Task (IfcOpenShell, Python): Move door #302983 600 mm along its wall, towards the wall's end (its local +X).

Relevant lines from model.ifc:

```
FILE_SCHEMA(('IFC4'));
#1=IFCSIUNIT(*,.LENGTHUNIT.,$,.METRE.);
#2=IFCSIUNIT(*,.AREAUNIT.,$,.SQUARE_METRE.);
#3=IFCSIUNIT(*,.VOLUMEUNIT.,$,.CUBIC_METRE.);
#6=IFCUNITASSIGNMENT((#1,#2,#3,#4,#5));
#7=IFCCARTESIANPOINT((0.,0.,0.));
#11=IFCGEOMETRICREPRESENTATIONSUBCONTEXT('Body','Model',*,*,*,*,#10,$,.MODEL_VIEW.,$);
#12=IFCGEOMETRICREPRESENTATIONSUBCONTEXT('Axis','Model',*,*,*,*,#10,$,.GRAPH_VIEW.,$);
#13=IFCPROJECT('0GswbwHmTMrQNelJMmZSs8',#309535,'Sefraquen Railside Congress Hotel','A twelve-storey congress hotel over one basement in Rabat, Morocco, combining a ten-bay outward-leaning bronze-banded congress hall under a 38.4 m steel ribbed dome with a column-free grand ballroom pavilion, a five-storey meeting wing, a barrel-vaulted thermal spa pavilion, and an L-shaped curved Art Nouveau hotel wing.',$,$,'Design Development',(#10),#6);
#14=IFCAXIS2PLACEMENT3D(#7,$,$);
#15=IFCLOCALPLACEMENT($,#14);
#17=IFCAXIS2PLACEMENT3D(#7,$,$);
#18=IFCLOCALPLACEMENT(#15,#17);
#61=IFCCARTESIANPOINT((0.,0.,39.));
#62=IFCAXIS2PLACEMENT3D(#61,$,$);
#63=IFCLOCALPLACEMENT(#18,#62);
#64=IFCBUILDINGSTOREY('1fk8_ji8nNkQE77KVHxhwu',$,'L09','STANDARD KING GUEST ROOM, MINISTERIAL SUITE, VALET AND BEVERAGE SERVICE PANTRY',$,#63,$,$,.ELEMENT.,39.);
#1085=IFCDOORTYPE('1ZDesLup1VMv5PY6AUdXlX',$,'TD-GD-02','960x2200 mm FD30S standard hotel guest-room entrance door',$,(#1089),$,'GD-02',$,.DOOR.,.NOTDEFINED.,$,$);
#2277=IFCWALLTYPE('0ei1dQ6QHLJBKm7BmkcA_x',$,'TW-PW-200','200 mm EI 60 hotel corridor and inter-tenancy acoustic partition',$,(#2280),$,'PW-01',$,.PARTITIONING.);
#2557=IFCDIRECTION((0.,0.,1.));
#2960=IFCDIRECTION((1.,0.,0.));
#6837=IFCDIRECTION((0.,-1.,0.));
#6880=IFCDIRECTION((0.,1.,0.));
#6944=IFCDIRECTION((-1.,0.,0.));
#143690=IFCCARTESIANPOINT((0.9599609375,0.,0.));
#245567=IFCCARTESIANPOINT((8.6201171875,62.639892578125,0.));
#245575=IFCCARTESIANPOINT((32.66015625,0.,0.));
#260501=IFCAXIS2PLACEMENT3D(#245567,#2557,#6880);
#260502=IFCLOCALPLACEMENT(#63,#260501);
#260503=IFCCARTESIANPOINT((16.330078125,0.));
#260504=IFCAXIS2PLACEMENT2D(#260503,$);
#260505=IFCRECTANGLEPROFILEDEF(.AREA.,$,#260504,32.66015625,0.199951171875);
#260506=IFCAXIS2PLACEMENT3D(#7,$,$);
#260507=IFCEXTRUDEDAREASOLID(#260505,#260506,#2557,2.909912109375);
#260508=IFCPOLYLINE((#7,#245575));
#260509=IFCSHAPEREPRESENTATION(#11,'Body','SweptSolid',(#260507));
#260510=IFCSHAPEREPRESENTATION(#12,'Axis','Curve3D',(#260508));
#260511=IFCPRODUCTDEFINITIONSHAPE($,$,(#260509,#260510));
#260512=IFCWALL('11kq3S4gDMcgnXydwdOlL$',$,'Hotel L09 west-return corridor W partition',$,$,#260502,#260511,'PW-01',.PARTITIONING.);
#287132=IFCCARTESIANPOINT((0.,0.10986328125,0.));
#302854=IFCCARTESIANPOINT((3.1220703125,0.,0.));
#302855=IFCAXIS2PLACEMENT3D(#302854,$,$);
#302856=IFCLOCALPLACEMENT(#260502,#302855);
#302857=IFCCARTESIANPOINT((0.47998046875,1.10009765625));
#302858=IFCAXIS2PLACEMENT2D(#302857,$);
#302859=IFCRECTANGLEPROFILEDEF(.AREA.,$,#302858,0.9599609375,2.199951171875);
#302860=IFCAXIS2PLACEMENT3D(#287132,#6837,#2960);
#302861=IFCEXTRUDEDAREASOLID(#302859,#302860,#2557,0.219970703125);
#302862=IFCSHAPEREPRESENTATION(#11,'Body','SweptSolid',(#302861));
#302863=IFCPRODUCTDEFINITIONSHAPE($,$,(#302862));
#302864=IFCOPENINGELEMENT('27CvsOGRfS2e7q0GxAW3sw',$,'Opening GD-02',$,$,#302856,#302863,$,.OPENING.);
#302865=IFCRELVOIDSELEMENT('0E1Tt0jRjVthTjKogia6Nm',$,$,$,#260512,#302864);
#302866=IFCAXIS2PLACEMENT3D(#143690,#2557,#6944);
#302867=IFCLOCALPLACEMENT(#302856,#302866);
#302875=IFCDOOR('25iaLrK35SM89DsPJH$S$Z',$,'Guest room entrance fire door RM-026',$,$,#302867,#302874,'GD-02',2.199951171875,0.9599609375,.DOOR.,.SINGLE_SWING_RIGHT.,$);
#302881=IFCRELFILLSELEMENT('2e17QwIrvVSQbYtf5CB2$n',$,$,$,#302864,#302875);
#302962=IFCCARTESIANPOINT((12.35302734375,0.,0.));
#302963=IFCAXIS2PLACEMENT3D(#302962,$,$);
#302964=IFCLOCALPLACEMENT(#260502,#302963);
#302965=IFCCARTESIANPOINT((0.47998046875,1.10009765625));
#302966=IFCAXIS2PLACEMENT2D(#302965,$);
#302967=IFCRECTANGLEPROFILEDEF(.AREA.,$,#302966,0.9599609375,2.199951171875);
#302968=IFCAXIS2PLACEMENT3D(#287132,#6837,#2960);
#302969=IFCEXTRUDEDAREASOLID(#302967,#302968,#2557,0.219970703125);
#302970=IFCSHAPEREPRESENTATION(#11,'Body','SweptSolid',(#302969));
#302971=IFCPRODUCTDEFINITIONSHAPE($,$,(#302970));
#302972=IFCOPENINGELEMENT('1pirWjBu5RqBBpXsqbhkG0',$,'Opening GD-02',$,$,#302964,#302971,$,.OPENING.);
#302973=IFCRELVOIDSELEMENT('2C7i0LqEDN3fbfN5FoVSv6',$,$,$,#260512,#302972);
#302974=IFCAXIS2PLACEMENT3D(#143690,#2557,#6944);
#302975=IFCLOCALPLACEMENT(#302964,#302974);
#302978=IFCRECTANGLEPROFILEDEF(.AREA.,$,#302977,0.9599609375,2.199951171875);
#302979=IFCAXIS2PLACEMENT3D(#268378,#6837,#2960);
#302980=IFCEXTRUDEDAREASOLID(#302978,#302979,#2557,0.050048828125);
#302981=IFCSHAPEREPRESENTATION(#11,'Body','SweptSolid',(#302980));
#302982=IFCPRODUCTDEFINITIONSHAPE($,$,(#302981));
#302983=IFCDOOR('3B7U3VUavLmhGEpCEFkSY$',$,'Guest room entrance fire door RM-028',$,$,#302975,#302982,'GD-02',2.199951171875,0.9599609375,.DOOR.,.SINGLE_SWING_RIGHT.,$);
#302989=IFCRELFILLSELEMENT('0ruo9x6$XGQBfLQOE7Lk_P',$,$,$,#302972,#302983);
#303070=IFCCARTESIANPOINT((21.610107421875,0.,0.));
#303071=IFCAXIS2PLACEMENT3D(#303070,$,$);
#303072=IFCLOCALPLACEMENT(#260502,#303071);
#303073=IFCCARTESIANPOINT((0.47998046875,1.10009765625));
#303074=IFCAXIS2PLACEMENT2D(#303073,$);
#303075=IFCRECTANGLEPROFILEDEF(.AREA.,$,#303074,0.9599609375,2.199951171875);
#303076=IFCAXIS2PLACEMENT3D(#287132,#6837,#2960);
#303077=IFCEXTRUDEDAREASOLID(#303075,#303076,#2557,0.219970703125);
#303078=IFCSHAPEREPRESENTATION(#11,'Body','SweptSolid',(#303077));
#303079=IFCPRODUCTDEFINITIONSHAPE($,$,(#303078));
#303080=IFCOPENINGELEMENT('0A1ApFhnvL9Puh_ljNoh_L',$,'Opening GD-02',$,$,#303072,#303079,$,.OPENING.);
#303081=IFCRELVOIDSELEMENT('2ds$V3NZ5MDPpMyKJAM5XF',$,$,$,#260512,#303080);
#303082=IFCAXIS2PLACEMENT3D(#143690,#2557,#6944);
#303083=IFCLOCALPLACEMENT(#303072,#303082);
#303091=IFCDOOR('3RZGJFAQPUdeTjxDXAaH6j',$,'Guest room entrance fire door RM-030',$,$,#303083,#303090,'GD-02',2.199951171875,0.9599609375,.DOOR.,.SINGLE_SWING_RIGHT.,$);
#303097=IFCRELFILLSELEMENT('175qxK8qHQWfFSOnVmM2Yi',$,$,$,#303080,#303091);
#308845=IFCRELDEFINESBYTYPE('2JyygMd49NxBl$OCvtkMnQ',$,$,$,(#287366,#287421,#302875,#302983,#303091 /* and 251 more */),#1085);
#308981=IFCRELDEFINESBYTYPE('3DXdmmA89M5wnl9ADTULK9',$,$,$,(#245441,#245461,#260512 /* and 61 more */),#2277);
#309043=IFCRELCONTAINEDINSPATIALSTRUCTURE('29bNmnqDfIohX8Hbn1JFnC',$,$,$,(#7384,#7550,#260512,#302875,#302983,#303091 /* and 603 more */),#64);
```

```python
import ifcopenshell
import ifcopenshell.api.geometry
import ifcopenshell.util.placement
import ifcopenshell.util.unit

model = ifcopenshell.open("model.ifc")
unit_scale = ifcopenshell.util.unit.calculate_unit_scale(model)

door = model.by_id(302983)
opening = door.FillsVoids[0].RelatingOpeningElement
wall = opening.VoidsElements[0].RelatingBuildingElement

wall_matrix = ifcopenshell.util.placement.get_local_placement(wall.ObjectPlacement)
shift = wall_matrix[:3, 0] * 0.6 / unit_scale
before = ifcopenshell.util.placement.get_local_placement(door.ObjectPlacement)[:3, 3].copy()

# The door is placed relative to its opening, so it follows when the opening moves.
matrix = ifcopenshell.util.placement.get_local_placement(opening.ObjectPlacement)
matrix[:3, 3] += shift
ifcopenshell.api.geometry.edit_object_placement(
    model, product=opening, matrix=matrix, is_si=False, should_transform_children=True
)

after = ifcopenshell.util.placement.get_local_placement(door.ObjectPlacement)[:3, 3]
print("door moved by", (after - before).round(3) + 0.0)

model.write("model_rev.ifc")
```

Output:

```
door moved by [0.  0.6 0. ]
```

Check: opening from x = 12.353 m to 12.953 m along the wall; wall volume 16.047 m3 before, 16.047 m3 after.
